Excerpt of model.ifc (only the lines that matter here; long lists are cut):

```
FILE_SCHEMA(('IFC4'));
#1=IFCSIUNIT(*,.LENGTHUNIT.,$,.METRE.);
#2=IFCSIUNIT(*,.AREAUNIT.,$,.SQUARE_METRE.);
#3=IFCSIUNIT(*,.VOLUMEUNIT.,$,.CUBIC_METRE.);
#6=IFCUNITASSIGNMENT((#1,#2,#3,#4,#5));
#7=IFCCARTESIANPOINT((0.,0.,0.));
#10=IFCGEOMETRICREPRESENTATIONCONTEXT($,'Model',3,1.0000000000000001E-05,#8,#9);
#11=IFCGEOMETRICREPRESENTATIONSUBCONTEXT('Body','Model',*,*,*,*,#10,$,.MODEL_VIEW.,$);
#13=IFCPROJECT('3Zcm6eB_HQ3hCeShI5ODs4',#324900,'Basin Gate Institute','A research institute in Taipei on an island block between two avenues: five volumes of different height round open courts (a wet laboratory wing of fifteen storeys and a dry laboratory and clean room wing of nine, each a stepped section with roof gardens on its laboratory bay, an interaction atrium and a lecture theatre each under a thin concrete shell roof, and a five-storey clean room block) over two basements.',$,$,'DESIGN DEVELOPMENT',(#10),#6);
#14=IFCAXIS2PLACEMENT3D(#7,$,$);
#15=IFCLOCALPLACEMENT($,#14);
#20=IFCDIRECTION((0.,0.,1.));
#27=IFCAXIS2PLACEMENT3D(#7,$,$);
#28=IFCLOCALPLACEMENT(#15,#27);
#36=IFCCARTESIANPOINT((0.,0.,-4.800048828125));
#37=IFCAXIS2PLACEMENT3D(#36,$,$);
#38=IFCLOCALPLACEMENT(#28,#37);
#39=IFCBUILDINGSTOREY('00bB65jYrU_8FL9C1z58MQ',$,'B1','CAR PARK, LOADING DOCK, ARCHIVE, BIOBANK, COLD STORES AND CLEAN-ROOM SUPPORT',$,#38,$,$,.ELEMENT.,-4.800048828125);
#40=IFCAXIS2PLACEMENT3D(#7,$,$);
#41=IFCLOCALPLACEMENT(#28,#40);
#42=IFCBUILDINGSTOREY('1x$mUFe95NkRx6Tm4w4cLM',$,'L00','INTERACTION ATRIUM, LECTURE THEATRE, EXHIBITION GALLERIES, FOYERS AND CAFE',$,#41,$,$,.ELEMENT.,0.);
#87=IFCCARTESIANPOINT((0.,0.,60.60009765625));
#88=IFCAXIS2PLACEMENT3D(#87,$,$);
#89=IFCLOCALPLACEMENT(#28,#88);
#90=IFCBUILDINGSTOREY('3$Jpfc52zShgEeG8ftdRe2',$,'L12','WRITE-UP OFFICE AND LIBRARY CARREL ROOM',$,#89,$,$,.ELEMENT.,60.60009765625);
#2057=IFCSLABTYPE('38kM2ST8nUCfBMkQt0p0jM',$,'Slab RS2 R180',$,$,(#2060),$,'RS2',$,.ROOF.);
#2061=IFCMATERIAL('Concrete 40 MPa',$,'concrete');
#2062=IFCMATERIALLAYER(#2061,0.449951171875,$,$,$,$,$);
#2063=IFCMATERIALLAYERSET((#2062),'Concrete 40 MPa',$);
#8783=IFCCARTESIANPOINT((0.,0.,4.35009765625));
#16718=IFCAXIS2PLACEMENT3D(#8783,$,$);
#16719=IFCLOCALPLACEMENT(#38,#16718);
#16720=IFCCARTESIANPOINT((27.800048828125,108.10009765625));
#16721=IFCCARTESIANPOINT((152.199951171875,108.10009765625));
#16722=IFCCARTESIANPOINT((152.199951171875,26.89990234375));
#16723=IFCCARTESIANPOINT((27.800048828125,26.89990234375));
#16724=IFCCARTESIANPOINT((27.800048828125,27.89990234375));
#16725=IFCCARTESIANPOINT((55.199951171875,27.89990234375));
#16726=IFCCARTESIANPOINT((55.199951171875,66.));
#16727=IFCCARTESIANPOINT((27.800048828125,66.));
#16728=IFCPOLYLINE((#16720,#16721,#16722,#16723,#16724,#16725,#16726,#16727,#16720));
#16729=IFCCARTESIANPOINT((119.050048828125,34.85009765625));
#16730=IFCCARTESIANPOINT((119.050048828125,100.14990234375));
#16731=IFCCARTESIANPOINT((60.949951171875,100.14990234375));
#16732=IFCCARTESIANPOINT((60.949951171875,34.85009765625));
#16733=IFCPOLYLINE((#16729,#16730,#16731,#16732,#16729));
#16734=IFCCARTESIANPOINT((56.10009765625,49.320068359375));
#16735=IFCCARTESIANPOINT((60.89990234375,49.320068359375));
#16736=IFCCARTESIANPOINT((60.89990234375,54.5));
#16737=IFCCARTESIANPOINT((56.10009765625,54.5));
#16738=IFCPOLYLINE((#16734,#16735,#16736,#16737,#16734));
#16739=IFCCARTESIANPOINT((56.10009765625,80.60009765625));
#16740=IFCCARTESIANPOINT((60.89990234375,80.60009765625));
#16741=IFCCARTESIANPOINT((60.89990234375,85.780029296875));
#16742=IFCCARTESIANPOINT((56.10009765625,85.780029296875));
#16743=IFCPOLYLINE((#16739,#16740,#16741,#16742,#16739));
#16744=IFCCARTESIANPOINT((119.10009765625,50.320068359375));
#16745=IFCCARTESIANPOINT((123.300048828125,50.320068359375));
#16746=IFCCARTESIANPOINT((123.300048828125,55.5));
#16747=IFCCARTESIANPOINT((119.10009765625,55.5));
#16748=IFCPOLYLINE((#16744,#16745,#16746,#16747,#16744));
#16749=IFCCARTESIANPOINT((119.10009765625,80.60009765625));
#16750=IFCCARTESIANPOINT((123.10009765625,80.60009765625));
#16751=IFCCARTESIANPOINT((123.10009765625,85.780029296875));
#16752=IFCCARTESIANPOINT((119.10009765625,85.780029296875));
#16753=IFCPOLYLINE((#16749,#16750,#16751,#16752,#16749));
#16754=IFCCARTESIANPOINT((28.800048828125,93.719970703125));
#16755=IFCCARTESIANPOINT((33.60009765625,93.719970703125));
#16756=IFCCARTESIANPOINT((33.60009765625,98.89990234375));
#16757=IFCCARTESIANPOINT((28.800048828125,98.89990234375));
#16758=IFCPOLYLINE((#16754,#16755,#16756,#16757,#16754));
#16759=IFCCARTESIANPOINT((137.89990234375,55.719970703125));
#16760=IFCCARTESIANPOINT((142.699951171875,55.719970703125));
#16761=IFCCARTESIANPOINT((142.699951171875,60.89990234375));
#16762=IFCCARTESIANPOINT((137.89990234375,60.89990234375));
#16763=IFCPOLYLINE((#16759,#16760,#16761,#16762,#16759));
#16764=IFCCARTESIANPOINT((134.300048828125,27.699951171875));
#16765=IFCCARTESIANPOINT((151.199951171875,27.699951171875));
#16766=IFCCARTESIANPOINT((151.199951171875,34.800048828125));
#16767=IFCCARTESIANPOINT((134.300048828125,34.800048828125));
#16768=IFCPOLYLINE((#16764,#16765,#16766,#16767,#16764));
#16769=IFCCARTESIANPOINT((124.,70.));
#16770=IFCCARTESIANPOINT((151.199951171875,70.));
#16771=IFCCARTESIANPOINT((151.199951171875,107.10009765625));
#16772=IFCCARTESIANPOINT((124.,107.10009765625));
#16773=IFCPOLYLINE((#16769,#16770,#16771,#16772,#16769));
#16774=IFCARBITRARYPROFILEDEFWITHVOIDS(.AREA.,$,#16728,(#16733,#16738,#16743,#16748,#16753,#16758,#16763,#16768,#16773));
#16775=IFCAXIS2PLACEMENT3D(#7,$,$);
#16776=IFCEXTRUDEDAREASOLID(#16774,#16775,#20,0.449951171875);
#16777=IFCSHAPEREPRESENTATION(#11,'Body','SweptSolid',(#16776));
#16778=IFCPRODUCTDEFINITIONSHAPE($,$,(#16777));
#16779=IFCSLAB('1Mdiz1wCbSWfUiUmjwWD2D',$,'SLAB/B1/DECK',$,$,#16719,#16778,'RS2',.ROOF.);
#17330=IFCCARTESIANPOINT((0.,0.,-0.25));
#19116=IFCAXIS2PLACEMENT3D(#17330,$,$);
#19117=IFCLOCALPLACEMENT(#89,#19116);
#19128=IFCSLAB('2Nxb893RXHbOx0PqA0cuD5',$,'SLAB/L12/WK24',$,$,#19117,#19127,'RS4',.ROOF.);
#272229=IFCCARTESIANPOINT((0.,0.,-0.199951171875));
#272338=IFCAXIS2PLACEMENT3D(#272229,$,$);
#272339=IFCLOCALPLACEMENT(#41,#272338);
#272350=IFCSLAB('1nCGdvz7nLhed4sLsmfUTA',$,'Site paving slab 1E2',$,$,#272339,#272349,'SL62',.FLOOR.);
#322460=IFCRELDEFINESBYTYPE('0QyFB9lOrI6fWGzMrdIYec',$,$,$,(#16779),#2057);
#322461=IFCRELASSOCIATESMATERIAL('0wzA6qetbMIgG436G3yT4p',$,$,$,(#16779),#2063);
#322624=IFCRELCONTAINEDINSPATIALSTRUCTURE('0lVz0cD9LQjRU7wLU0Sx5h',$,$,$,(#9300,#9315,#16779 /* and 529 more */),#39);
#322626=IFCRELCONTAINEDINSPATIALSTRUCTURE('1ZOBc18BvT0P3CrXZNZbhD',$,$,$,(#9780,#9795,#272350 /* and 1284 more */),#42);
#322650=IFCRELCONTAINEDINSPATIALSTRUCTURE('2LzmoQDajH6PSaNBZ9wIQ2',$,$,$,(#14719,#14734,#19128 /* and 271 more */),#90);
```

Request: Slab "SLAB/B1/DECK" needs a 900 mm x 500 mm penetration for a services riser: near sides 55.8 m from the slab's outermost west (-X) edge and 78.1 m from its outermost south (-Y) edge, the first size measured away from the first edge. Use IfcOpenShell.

```python
import numpy as np
import ifcopenshell
import ifcopenshell.api.feature
import ifcopenshell.api.geometry
import ifcopenshell.api.root
import ifcopenshell.geom
import ifcopenshell.util.placement
import ifcopenshell.util.representation
import ifcopenshell.util.shape
import ifcopenshell.util.unit

model = ifcopenshell.open("model.ifc")
unit_scale = ifcopenshell.util.unit.calculate_unit_scale(model)
settings = ifcopenshell.geom.settings()


def volume(element):
    """Net volume in cubic metres, openings subtracted."""
    shape = ifcopenshell.geom.create_shape(settings, element)
    return ifcopenshell.util.shape.get_volume(shape.geometry)


slab = model.by_guid("1Mdiz1wCbSWfUiUmjwWD2D")
before = volume(slab)

# Extent in the slab's own axes, in metres. The edges named are its -X and -Y sides.
slab_shape = ifcopenshell.geom.create_shape(settings, slab)
vertices = ifcopenshell.util.shape.get_vertices(slab_shape.geometry)
x_min, y_min, bottom = vertices.min(axis=0)
top = vertices[:, 2].max()

opening = ifcopenshell.api.root.create_entity(model, ifc_class="IfcOpeningElement", name="Services riser opening", predefined_type="OPENING")
context = ifcopenshell.util.representation.get_context(model, "Model", "Body", "MODEL_VIEW")
width, depth = 0.9, 0.5
outline = [(0.0, 0.0), (width, 0.0), (width, depth), (0.0, depth), (0.0, 0.0)]
# Overshoot both faces by 50 mm so the cut is clean.
shape = ifcopenshell.api.geometry.add_slab_representation(
    model, context=context, depth=top - bottom + 0.1, polyline=outline
)
ifcopenshell.api.geometry.assign_representation(model, product=opening, representation=shape)

matrix = ifcopenshell.util.placement.get_local_placement(slab.ObjectPlacement)
matrix[:, 3] = matrix @ np.append(np.array([x_min + 55.8, y_min + 78.1, bottom - 0.05]) / unit_scale, 1.0)
ifcopenshell.api.geometry.edit_object_placement(model, product=opening, matrix=matrix, is_si=False)
ifcopenshell.api.feature.add_feature(model, feature=opening, element=slab)

after = volume(slab)

print(f"slab volume {before:.3f} -> {after:.3f} m3")

model.write("model_updated.ifc")
```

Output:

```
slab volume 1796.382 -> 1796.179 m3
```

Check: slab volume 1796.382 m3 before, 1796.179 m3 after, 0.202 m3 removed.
